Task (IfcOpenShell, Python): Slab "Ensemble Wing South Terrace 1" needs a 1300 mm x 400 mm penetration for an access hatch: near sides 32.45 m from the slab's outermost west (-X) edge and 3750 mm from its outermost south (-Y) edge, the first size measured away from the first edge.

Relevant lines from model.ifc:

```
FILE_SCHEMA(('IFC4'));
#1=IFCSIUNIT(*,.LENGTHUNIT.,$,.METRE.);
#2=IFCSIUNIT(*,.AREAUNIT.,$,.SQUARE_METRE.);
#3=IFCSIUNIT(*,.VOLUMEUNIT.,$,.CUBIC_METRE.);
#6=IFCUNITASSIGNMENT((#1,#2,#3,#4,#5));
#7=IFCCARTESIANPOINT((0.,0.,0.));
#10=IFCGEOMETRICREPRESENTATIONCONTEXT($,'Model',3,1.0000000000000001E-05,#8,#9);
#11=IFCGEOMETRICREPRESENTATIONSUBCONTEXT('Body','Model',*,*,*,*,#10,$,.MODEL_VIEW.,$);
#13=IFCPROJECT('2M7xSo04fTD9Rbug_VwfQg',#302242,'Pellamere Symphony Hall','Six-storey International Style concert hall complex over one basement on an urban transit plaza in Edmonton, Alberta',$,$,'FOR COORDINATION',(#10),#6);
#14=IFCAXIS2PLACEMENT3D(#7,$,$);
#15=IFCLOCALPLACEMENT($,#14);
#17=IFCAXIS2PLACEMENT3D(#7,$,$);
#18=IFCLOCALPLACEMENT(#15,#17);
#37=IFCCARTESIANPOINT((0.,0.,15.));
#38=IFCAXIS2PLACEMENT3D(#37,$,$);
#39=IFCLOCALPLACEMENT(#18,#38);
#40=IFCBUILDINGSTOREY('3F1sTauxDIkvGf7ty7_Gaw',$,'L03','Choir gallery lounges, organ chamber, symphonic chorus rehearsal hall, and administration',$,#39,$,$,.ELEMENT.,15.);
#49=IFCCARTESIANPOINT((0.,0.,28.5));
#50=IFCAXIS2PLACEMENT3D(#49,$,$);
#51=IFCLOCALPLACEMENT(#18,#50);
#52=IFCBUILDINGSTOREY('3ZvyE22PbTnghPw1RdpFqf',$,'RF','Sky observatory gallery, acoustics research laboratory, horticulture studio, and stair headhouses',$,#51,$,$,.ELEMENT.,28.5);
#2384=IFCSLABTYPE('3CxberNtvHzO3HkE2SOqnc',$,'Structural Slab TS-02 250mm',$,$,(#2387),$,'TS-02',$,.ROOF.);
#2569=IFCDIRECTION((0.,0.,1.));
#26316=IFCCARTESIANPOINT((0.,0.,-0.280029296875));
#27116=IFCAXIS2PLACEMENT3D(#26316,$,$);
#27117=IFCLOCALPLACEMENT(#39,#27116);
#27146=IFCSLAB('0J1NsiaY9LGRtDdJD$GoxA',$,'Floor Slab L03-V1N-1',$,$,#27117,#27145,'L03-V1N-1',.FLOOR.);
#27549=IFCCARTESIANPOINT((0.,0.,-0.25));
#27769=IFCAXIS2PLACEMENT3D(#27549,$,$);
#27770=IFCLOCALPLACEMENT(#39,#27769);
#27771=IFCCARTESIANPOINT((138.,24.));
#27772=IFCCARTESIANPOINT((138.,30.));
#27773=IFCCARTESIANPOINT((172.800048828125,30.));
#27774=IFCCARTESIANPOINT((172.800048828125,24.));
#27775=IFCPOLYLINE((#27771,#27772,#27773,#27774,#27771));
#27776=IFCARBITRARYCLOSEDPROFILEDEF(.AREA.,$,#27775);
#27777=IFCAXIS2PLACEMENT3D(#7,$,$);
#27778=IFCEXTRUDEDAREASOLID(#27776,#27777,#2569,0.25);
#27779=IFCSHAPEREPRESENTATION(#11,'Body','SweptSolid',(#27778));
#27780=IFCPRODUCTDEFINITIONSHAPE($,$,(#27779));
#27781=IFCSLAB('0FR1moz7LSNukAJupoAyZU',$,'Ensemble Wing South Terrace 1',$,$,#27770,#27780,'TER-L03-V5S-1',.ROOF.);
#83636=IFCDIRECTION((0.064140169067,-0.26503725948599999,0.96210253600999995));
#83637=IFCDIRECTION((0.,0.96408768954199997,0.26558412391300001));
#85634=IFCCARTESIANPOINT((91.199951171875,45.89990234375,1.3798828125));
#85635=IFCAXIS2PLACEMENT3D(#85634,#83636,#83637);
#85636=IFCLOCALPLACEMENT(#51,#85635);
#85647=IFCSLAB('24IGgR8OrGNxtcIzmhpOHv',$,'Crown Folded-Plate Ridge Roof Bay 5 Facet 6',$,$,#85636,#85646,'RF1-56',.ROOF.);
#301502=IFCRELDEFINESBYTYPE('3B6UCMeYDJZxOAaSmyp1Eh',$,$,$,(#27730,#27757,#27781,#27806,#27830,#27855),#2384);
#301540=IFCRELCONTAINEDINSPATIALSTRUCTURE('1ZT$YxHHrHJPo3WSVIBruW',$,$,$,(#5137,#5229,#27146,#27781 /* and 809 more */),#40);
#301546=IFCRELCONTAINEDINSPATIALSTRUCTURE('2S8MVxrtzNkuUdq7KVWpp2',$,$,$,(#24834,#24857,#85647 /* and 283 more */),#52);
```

```python
import numpy as np
import ifcopenshell
import ifcopenshell.api.feature
import ifcopenshell.api.geometry
import ifcopenshell.api.root
import ifcopenshell.geom
import ifcopenshell.util.placement
import ifcopenshell.util.representation
import ifcopenshell.util.shape
import ifcopenshell.util.unit

model = ifcopenshell.open("model.ifc")
unit_scale = ifcopenshell.util.unit.calculate_unit_scale(model)
settings = ifcopenshell.geom.settings()


def volume(element):
    """Net volume in cubic metres, openings subtracted."""
    shape = ifcopenshell.geom.create_shape(settings, element)
    return ifcopenshell.util.shape.get_volume(shape.geometry)


slab = model.by_guid("0FR1moz7LSNukAJupoAyZU")
before = volume(slab)

# Extent in the slab's own axes, in metres. The edges named are its -X and -Y sides.
slab_shape = ifcopenshell.geom.create_shape(settings, slab)
vertices = ifcopenshell.util.shape.get_vertices(slab_shape.geometry)
x_min, y_min, bottom = vertices.min(axis=0)
top = vertices[:, 2].max()

opening = ifcopenshell.api.root.create_entity(model, ifc_class="IfcOpeningElement", name="Access hatch opening", predefined_type="OPENING")
context = ifcopenshell.util.representation.get_context(model, "Model", "Body", "MODEL_VIEW")
width, depth = 1.3, 0.4
outline = [(0.0, 0.0), (width, 0.0), (width, depth), (0.0, depth), (0.0, 0.0)]
# Overshoot both faces by 50 mm so the cut is clean.
shape = ifcopenshell.api.geometry.add_slab_representation(
    model, context=context, depth=top - bottom + 0.1, polyline=outline
)
ifcopenshell.api.geometry.assign_representation(model, product=opening, representation=shape)

matrix = ifcopenshell.util.placement.get_local_placement(slab.ObjectPlacement)
matrix[:, 3] = matrix @ np.append(np.array([x_min + 32.45, y_min + 3.75, bottom - 0.05]) / unit_scale, 1.0)
ifcopenshell.api.geometry.edit_object_placement(model, product=opening, matrix=matrix, is_si=False)
ifcopenshell.api.feature.add_feature(model, feature=opening, element=slab)

after = volume(slab)

print(f"slab volume {before:.3f} -> {after:.3f} m3")

model.write("model-out.ifc")
```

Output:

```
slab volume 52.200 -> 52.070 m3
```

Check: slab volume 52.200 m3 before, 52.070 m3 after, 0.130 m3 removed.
